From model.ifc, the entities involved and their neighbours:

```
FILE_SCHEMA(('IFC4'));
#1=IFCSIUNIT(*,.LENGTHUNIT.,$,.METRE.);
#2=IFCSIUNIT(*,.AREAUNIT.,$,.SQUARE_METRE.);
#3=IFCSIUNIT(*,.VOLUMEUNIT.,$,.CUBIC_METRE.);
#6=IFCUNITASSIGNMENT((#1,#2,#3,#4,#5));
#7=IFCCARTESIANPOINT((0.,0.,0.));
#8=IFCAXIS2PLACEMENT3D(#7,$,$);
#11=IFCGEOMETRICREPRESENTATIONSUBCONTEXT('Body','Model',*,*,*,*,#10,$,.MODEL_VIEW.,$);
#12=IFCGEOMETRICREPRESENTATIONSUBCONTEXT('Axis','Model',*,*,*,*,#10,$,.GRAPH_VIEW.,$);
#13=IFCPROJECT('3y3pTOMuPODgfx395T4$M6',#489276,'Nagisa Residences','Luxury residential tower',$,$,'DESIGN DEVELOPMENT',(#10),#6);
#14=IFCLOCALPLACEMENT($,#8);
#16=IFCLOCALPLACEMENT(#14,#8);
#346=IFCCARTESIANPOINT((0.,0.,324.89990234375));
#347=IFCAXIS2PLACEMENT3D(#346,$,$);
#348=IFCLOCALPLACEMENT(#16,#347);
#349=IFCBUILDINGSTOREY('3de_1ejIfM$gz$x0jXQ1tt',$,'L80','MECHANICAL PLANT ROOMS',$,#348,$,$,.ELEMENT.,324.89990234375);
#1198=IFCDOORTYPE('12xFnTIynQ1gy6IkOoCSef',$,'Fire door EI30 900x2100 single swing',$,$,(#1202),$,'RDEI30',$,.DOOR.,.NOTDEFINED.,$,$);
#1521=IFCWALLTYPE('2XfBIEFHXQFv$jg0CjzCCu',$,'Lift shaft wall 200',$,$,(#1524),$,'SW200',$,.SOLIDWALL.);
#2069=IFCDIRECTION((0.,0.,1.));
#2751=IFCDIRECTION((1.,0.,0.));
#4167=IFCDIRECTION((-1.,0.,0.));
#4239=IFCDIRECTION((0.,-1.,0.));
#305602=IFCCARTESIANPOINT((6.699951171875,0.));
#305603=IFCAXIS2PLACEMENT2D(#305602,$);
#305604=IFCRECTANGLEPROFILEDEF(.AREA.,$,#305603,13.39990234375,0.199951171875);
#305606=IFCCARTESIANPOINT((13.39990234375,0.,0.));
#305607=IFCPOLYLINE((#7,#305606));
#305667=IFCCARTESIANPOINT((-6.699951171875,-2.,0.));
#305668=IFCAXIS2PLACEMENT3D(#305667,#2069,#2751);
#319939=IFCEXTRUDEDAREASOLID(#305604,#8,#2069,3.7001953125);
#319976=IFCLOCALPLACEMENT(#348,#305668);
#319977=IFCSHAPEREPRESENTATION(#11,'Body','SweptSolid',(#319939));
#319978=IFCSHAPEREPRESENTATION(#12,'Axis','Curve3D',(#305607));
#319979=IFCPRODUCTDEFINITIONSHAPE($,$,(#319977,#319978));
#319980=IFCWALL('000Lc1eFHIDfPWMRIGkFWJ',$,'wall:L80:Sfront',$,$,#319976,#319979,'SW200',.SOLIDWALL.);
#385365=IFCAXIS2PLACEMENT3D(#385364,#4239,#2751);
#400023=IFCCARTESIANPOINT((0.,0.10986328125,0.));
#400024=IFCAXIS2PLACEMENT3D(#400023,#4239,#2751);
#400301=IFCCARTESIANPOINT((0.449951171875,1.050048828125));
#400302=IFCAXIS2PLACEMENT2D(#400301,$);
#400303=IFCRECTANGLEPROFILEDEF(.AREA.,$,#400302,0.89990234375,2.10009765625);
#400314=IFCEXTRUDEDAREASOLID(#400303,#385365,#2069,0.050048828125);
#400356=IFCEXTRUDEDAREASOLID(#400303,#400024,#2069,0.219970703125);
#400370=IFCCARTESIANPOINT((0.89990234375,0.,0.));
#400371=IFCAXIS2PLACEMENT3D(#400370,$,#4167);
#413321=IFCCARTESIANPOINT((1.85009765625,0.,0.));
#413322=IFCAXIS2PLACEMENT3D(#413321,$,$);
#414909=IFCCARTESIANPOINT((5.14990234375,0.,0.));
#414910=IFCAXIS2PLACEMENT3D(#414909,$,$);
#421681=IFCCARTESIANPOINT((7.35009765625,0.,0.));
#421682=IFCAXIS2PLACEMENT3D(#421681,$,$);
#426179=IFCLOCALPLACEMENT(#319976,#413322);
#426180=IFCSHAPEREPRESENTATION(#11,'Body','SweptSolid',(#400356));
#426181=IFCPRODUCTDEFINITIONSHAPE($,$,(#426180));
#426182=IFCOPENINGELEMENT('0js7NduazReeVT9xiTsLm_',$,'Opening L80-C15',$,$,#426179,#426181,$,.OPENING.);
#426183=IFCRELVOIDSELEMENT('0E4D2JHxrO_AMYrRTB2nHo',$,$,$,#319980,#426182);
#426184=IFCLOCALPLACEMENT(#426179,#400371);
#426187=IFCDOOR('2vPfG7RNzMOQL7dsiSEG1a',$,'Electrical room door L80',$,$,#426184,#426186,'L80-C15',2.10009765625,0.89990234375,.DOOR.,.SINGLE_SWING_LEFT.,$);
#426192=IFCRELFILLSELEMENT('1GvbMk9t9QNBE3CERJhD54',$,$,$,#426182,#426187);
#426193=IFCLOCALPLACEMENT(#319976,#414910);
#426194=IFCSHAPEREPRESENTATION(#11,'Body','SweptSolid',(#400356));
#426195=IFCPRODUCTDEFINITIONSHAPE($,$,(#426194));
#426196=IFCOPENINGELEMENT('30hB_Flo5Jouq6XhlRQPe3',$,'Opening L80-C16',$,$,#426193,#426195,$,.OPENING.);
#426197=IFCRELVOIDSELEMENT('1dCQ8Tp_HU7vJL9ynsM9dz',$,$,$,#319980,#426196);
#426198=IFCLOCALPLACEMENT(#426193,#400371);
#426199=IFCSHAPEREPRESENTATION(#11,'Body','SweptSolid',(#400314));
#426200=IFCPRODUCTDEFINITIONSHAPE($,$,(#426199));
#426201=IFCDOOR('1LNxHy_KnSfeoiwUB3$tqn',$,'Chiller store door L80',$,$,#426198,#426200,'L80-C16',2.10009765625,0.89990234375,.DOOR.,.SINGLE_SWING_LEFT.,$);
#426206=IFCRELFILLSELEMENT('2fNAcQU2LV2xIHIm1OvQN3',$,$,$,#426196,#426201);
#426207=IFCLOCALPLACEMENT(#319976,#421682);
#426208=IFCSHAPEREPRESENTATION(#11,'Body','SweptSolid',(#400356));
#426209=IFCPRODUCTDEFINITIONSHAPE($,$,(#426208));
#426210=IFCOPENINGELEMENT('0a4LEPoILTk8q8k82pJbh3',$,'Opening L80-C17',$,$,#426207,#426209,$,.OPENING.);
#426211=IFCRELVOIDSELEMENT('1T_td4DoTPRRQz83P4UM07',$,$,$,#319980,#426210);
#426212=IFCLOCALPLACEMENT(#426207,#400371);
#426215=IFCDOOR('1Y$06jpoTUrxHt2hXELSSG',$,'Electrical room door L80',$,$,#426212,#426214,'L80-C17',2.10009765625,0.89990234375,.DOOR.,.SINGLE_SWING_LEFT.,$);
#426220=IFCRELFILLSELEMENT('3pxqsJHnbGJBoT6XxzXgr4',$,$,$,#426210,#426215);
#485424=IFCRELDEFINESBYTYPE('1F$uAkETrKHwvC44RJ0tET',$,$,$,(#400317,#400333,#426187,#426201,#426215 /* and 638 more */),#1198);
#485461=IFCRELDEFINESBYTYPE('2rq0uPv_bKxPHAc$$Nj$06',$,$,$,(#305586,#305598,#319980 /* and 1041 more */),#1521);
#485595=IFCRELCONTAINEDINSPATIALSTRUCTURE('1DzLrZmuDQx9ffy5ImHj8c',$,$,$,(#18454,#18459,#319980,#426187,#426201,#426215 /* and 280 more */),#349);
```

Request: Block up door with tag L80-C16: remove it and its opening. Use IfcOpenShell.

```python
import ifcopenshell
import ifcopenshell.api.feature
import ifcopenshell.api.root
import ifcopenshell.geom
import ifcopenshell.util.shape

model = ifcopenshell.open("model.ifc")
settings = ifcopenshell.geom.settings()


def volume(element):
    """Net volume in cubic metres, openings subtracted."""
    shape = ifcopenshell.geom.create_shape(settings, element)
    return ifcopenshell.util.shape.get_volume(shape.geometry)


door = model.by_guid("1LNxHy_KnSfeoiwUB3$tqn")
opening = door.FillsVoids[0].RelatingOpeningElement
wall = opening.VoidsElements[0].RelatingBuildingElement
before = volume(wall)

ifcopenshell.api.root.remove_product(model, product=door)
ifcopenshell.api.feature.remove_feature(model, feature=opening)

after = volume(wall)

print(f"wall volume {before:.3f} -> {after:.3f} m3")

model.write("model_v2.ifc")
```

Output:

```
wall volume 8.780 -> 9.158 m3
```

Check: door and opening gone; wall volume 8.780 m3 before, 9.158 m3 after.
